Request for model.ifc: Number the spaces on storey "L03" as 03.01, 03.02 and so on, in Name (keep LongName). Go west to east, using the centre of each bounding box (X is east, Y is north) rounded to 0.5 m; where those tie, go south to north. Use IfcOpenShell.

First a look at what the model holds.

```python
import ifcopenshell
import ifcopenshell.util.element
import ifcopenshell.util.placement

model = ifcopenshell.open("model.ifc")
print(model.schema)
storey = next(s for s in model.by_type("IfcBuildingStorey") if s.Name == "L03")
spaces = [e for e in ifcopenshell.util.element.get_decomposition(storey) if e.is_a("IfcSpace")]
for e in sorted(spaces, key=lambda e: e.id()):
    origin = ifcopenshell.util.placement.get_local_placement(e.ObjectPlacement)[:3, 3]
    print(e.id(), e.Name, e.LongName, origin.round(2) + 0.0, sep=" | ")
```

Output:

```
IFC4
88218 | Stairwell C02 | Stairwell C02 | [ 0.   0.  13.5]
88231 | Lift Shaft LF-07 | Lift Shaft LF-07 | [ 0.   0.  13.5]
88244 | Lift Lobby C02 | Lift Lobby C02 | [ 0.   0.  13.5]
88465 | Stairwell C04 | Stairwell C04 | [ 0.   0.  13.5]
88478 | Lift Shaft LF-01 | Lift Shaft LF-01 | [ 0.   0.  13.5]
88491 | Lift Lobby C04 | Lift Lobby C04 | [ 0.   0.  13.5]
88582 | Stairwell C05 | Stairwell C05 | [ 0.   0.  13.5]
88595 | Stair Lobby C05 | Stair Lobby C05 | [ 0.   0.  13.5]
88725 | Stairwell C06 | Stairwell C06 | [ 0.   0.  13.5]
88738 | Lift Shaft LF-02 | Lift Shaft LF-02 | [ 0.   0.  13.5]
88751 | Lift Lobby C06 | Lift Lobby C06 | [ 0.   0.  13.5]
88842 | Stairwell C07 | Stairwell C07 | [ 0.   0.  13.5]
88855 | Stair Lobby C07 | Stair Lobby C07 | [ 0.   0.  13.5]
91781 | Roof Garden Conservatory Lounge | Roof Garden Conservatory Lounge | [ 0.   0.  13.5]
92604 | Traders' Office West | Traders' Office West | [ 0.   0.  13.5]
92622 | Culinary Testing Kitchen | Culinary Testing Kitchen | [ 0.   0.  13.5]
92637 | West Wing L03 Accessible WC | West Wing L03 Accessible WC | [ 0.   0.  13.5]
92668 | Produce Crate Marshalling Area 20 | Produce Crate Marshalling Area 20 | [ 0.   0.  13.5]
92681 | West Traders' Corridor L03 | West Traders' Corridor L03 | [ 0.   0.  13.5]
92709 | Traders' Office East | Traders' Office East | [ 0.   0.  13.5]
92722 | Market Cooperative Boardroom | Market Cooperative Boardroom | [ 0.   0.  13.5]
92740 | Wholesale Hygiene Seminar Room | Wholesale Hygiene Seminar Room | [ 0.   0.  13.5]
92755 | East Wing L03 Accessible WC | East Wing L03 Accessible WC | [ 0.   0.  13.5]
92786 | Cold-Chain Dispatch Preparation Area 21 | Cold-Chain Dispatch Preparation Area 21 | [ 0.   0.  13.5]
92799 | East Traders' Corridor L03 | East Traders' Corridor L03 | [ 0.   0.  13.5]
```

```python
import ifcopenshell
import ifcopenshell.geom
import ifcopenshell.util.element
import ifcopenshell.util.shape

model = ifcopenshell.open("model.ifc")
settings = ifcopenshell.geom.settings()
settings.set("use-world-coords", True)


def centre(element):
    shape = ifcopenshell.geom.create_shape(settings, element)
    return ifcopenshell.util.shape.get_bbox_centroid(shape.geometry)


storey = next(s for s in model.by_type("IfcBuildingStorey") if s.Name == "L03")
spaces = [e for e in ifcopenshell.util.element.get_decomposition(storey) if e.is_a("IfcSpace")]

# Insertion points can sit at a corner or the storey origin, so sort by the geometry (in metres).
centres = {e: centre(e) for e in spaces}
spaces.sort(key=lambda e: (round(centres[e][0] / 0.5), centres[e][1]))

for i, e in enumerate(spaces, start=1):
    number = f"03.{i:02d}"
    e.Name = number
    print(e.id(), number)

model.write("model_updated.ifc")
```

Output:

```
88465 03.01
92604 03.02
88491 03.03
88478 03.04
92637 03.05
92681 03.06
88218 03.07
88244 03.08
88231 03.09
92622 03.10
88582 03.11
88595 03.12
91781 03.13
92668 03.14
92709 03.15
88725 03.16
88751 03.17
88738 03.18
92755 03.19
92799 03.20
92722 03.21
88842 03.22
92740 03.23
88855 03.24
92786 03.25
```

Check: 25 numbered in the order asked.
